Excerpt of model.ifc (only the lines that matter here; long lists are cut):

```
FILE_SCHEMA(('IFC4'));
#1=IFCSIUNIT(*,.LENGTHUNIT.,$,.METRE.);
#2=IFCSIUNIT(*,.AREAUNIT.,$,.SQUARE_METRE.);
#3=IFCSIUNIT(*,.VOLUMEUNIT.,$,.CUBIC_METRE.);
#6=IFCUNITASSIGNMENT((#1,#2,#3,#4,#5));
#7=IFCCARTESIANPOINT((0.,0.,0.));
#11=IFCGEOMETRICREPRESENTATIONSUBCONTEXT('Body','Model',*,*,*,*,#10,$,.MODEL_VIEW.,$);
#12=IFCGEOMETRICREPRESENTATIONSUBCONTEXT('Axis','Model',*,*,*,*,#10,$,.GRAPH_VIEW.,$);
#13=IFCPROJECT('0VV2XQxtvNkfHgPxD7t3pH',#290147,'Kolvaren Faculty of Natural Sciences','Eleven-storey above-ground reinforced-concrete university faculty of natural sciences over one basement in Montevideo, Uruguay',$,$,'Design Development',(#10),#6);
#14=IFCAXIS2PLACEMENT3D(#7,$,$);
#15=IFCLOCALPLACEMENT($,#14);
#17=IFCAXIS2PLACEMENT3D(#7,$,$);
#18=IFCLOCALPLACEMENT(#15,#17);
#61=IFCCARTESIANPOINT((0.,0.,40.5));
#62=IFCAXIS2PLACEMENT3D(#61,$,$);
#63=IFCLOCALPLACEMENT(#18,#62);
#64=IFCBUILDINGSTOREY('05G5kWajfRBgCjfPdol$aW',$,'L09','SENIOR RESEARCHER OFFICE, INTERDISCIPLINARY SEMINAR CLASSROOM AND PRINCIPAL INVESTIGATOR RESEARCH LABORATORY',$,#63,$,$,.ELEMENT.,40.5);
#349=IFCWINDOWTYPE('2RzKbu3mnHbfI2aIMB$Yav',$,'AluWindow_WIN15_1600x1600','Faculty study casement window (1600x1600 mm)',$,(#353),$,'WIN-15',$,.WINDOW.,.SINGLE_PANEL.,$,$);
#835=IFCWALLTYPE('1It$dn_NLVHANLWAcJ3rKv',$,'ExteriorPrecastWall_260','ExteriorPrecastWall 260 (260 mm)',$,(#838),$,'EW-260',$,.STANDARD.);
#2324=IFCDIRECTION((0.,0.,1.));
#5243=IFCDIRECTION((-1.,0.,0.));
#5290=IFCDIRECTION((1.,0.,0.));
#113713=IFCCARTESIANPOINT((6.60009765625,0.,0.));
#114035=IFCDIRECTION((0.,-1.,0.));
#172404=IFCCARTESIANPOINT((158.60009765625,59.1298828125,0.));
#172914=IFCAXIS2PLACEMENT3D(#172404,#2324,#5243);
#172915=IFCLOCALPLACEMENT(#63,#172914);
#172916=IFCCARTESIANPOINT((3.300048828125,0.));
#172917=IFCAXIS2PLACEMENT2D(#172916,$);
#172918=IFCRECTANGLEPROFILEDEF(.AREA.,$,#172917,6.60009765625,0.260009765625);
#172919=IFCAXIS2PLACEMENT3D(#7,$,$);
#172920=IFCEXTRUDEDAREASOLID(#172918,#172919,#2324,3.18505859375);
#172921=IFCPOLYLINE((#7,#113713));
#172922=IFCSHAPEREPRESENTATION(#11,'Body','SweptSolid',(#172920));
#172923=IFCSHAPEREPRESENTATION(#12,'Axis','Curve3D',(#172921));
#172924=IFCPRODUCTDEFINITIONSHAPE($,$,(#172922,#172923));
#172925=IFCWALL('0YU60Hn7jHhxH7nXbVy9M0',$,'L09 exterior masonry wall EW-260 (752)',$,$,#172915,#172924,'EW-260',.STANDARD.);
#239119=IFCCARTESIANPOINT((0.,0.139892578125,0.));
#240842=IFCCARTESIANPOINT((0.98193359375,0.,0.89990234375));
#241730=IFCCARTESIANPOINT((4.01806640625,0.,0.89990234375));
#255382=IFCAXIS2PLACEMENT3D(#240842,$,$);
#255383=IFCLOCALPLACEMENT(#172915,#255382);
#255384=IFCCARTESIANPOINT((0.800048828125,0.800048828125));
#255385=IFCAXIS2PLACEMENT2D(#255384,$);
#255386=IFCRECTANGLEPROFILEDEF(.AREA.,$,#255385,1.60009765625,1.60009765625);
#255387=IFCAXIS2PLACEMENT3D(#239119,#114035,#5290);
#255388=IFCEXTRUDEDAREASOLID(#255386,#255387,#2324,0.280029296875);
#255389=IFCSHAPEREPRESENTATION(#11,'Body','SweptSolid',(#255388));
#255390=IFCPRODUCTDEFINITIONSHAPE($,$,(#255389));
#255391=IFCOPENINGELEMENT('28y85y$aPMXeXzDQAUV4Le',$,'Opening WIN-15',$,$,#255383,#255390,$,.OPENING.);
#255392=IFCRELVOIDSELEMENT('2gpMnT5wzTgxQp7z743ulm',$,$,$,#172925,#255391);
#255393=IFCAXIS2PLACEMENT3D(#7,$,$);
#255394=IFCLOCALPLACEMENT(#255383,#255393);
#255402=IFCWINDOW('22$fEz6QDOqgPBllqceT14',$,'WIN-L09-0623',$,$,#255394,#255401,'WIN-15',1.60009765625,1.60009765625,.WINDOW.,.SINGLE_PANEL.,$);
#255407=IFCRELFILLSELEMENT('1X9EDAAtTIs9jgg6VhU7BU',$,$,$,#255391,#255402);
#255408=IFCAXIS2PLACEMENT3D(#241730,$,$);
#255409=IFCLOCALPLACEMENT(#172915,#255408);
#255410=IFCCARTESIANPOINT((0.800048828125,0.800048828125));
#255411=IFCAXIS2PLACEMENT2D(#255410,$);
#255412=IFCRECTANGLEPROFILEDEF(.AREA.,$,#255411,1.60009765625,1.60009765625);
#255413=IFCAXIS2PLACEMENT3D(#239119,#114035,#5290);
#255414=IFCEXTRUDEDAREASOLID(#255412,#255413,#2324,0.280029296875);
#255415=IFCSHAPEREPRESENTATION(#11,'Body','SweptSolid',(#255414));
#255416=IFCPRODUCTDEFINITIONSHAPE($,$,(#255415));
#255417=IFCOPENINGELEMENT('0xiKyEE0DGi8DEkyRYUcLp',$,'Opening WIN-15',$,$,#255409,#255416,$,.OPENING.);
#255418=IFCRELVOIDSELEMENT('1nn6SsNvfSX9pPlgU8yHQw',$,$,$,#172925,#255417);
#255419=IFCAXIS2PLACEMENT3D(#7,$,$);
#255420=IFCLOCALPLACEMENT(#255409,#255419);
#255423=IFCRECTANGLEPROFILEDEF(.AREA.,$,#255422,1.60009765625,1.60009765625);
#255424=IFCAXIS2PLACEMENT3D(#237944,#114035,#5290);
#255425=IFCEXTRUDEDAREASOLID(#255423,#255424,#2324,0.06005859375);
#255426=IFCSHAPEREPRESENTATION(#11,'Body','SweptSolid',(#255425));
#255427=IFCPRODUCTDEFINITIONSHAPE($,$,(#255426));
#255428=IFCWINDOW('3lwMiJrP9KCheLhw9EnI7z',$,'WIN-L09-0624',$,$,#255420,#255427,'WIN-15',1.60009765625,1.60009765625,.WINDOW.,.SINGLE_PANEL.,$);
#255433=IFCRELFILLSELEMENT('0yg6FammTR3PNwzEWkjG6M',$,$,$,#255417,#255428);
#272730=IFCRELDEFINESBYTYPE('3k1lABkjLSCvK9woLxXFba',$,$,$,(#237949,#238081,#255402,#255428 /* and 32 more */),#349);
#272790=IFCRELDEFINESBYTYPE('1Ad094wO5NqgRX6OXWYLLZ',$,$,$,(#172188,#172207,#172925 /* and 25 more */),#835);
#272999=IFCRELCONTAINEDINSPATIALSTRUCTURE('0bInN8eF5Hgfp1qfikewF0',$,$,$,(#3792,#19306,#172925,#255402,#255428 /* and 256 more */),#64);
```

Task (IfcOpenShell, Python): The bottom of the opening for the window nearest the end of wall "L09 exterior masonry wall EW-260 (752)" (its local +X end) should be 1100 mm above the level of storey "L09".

```python
import numpy as np
import ifcopenshell
import ifcopenshell.api.geometry
import ifcopenshell.geom
import ifcopenshell.util.element
import ifcopenshell.util.placement
import ifcopenshell.util.shape
import ifcopenshell.util.unit

model = ifcopenshell.open("model.ifc")
unit_scale = ifcopenshell.util.unit.calculate_unit_scale(model)

window = model.by_guid("3lwMiJrP9KCheLhw9EnI7z")
opening = window.FillsVoids[0].RelatingOpeningElement
storey = ifcopenshell.util.element.get_container(window, ifc_class="IfcBuildingStorey")
level = ifcopenshell.util.placement.get_local_placement(storey.ObjectPlacement)[2, 3]

# The opening's origin need not be at the sill, so measure its lowest point.
shape = ifcopenshell.geom.create_shape(ifcopenshell.geom.settings(), opening)
bottom = ifcopenshell.util.shape.get_shape_bottom_elevation(shape, shape.geometry) / unit_scale
dz = level + 1.1 - bottom

shift = np.array([0.0, 0.0, dz])
# The window is placed relative to its opening, so it follows when the opening moves.
matrix = ifcopenshell.util.placement.get_local_placement(opening.ObjectPlacement)
matrix[:3, 3] += shift
ifcopenshell.api.geometry.edit_object_placement(
    model, product=opening, matrix=matrix, is_si=False, should_transform_children=True
)

print(f"moved by {dz * unit_scale:+.3f} m")

model.write("model_updated.ifc")
```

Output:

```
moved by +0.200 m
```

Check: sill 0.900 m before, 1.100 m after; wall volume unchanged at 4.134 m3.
